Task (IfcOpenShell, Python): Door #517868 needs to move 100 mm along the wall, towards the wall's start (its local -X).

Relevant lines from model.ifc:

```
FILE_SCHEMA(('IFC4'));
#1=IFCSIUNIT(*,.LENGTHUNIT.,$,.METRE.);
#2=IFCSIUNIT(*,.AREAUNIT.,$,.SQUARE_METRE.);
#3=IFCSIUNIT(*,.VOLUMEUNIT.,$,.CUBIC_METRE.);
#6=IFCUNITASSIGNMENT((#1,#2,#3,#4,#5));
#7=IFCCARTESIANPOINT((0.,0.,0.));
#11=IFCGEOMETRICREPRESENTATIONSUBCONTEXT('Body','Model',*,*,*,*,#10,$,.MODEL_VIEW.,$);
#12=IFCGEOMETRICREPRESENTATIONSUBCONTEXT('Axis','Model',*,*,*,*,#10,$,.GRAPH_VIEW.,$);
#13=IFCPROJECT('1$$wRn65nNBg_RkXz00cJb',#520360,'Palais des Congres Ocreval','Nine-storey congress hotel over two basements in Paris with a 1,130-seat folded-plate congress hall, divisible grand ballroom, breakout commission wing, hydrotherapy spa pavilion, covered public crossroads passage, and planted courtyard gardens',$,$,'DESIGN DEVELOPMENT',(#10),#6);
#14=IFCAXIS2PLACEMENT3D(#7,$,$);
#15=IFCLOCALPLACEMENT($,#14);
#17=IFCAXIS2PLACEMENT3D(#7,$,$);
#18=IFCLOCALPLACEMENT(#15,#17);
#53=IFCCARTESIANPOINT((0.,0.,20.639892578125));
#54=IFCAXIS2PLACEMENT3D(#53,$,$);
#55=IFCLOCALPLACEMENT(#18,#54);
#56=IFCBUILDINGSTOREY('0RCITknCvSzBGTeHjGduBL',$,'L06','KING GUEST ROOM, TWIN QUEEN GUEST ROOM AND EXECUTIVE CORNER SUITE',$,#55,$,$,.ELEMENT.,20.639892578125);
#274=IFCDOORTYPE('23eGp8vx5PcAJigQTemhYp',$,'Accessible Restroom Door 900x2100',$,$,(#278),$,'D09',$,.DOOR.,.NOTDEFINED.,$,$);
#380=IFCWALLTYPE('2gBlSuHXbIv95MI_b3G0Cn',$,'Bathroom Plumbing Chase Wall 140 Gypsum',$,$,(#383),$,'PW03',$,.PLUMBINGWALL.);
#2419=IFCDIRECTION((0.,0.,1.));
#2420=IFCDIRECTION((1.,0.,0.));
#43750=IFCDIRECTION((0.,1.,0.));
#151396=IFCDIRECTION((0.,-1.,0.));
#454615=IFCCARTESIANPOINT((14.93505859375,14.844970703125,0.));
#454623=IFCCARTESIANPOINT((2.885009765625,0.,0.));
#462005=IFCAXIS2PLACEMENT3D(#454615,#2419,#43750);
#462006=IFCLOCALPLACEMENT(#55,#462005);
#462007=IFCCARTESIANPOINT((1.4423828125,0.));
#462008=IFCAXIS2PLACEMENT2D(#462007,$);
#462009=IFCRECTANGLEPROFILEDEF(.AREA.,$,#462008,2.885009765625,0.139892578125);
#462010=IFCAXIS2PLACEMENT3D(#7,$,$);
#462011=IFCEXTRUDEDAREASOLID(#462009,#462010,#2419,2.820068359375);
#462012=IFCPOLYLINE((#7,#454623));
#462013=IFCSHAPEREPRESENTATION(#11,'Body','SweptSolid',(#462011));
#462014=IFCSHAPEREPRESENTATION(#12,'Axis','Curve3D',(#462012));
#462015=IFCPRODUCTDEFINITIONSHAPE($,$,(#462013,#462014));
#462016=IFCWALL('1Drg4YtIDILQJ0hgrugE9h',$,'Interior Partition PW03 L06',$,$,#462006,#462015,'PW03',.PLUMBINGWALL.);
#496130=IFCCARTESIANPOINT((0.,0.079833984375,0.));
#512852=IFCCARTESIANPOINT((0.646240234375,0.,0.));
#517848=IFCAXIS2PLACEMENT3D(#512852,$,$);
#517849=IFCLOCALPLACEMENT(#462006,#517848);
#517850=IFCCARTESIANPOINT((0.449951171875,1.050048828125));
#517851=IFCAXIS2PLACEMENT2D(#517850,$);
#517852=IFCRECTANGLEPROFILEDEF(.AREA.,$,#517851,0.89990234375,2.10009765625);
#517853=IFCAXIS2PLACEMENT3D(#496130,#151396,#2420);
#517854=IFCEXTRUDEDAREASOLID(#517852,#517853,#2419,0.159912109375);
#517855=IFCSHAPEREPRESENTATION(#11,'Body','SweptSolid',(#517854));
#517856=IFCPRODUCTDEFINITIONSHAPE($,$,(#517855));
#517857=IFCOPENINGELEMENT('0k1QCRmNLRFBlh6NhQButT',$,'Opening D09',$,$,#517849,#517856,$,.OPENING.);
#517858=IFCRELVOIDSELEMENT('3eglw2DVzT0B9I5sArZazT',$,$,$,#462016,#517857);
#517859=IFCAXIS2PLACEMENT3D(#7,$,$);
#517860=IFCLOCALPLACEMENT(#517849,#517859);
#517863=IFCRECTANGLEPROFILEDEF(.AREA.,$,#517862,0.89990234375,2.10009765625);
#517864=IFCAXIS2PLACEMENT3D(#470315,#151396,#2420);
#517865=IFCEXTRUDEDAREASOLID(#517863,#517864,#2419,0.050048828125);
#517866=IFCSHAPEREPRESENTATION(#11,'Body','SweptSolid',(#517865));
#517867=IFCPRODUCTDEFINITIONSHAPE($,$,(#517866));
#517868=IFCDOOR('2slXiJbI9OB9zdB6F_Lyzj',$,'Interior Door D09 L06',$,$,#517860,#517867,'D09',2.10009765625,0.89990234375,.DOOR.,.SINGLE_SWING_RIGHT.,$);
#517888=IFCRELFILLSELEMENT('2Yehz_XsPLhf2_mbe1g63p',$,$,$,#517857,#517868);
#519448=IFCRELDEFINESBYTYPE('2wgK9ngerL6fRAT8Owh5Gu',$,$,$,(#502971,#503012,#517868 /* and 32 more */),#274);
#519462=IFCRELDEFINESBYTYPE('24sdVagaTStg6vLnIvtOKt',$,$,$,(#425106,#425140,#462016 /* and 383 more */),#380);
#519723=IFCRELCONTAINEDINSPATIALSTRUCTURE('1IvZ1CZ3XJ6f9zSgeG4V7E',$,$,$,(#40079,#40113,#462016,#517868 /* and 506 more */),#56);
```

```python
import ifcopenshell
import ifcopenshell.api.geometry
import ifcopenshell.util.placement

model = ifcopenshell.open("model.ifc")

door = model.by_id(517868)
opening = door.FillsVoids[0].RelatingOpeningElement
wall = opening.VoidsElements[0].RelatingBuildingElement

wall_matrix = ifcopenshell.util.placement.get_local_placement(wall.ObjectPlacement)
shift = wall_matrix[:3, 0] * -0.1
before = ifcopenshell.util.placement.get_local_placement(door.ObjectPlacement)[:3, 3].copy()

# The door is placed relative to its opening, so it follows when the opening moves.
matrix = ifcopenshell.util.placement.get_local_placement(opening.ObjectPlacement)
matrix[:3, 3] += shift
ifcopenshell.api.geometry.edit_object_placement(
    model, product=opening, matrix=matrix, is_si=False, should_transform_children=True
)

after = ifcopenshell.util.placement.get_local_placement(door.ObjectPlacement)[:3, 3]
print("door moved by", (after - before).round(3) + 0.0)

model.write("model_v2.ifc")
```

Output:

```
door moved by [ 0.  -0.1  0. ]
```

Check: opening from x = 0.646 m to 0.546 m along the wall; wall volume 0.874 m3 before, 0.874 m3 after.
